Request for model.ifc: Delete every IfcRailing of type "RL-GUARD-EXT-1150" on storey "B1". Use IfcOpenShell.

First a look at what the model holds.

```python
import ifcopenshell
import ifcopenshell.util.element

model = ifcopenshell.open("model.ifc")
print(model.schema)
storey = next(s for s in model.by_type("IfcBuildingStorey") if s.Name == "B1")
railings = [e for e in ifcopenshell.util.element.get_decomposition(storey) if e.is_a("IfcRailing")]
seen = {}
for e in railings:
    element_type = ifcopenshell.util.element.get_type(e)
    name = element_type.Name if element_type not in (None, e) else None
    seen[name] = seen.get(name, 0) + 1
for name, count in sorted(seen.items(), key=str):
    print(count, "x", name)
```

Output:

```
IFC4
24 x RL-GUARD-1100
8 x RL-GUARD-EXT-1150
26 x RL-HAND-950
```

```python
import ifcopenshell
import ifcopenshell.api.root
import ifcopenshell.util.element

model = ifcopenshell.open("model.ifc")

storey = next(s for s in model.by_type("IfcBuildingStorey") if s.Name == "B1")
railings = [e for e in ifcopenshell.util.element.get_decomposition(storey) if e.is_a("IfcRailing")]
targets = [e for e in railings if (t := ifcopenshell.util.element.get_type(e)) not in (None, e) and t.Name == "RL-GUARD-EXT-1150"]

for e in targets:
    ifcopenshell.api.root.remove_product(model, product=e)
print(len(targets), "removed")

model.write("model_rev.ifc")
```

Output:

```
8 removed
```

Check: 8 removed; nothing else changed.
